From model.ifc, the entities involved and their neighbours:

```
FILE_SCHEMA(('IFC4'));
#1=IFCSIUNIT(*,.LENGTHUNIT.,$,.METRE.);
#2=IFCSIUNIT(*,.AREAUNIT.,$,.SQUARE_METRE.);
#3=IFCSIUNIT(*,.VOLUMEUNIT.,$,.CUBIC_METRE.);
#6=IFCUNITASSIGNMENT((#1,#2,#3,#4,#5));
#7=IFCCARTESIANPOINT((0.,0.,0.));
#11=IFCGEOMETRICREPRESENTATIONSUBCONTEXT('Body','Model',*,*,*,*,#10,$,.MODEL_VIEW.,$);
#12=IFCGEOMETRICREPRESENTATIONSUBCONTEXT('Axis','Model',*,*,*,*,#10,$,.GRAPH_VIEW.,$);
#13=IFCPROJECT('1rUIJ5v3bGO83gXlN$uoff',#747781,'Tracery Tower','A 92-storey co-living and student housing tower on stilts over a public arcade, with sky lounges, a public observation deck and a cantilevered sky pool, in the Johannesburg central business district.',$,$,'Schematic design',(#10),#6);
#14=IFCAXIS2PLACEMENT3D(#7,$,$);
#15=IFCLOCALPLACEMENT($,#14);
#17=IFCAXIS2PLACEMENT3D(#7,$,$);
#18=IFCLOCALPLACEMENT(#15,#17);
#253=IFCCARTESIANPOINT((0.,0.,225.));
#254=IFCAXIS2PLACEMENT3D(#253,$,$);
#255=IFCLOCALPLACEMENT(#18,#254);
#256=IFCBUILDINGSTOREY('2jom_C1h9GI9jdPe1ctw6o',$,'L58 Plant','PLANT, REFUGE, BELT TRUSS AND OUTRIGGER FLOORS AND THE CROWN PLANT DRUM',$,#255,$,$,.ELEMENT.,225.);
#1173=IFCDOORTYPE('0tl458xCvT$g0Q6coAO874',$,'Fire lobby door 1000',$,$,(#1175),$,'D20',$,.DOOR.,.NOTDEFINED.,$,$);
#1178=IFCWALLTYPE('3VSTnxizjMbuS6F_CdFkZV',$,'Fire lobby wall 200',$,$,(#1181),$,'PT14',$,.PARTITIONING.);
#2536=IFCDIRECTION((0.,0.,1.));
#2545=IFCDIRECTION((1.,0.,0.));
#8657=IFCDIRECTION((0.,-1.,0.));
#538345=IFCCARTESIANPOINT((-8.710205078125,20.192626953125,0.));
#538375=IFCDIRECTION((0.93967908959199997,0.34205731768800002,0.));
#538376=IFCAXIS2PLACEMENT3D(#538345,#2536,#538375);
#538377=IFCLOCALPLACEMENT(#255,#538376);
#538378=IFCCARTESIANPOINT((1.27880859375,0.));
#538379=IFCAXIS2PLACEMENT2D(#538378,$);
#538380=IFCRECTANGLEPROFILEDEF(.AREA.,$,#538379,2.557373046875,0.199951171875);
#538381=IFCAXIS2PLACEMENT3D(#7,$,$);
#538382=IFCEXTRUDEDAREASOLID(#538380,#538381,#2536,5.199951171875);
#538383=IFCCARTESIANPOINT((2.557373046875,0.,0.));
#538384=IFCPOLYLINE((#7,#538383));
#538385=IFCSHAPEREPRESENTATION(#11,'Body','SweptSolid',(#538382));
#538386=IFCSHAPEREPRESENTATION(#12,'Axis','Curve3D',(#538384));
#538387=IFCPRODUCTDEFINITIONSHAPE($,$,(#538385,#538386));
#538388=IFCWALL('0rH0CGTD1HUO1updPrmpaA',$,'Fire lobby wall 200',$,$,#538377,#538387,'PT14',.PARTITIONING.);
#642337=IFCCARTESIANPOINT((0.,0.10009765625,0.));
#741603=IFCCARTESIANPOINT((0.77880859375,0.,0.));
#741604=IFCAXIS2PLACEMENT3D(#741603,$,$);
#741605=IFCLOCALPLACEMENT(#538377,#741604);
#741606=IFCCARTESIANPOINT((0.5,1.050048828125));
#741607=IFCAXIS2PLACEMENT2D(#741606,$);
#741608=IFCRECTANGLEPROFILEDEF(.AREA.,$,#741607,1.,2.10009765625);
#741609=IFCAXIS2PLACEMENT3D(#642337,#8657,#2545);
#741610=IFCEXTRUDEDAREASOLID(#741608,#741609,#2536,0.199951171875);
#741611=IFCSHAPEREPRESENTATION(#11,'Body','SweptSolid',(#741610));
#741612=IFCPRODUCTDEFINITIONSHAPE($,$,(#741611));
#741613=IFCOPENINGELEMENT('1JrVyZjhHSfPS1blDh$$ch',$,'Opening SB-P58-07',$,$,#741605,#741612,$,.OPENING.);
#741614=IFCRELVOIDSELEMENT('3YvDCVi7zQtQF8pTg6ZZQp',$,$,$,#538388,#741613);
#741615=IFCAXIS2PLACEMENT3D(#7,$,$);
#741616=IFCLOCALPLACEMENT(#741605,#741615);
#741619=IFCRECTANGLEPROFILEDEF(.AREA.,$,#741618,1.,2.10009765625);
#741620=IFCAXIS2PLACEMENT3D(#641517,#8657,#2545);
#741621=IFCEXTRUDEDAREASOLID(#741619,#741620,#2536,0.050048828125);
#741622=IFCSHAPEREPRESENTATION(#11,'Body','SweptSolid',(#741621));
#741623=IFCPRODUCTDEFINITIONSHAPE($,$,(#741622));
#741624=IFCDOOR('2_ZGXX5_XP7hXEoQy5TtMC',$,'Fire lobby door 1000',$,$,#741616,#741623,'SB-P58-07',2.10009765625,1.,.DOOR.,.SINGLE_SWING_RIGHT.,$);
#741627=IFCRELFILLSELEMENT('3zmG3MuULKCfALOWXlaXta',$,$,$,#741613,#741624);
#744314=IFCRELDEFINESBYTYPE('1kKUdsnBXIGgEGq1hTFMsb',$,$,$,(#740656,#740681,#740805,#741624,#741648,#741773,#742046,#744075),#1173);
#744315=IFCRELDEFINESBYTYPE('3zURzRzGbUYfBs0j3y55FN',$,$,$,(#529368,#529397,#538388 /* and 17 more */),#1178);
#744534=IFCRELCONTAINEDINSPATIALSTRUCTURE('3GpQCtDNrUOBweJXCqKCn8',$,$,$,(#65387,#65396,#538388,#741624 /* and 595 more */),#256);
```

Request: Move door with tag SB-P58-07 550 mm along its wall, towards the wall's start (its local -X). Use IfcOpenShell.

```python
import ifcopenshell
import ifcopenshell.api.geometry
import ifcopenshell.util.placement
import ifcopenshell.util.unit

model = ifcopenshell.open("model.ifc")
unit_scale = ifcopenshell.util.unit.calculate_unit_scale(model)

door = model.by_id(741624)
opening = door.FillsVoids[0].RelatingOpeningElement
wall = opening.VoidsElements[0].RelatingBuildingElement

wall_matrix = ifcopenshell.util.placement.get_local_placement(wall.ObjectPlacement)
shift = wall_matrix[:3, 0] * -0.55 / unit_scale
before = ifcopenshell.util.placement.get_local_placement(door.ObjectPlacement)[:3, 3].copy()

# The door is placed relative to its opening, so it follows when the opening moves.
matrix = ifcopenshell.util.placement.get_local_placement(opening.ObjectPlacement)
matrix[:3, 3] += shift
ifcopenshell.api.geometry.edit_object_placement(
    model, product=opening, matrix=matrix, is_si=False, should_transform_children=True
)

after = ifcopenshell.util.placement.get_local_placement(door.ObjectPlacement)[:3, 3]
print("door moved by", (after - before).round(3) + 0.0)

model.write("model_v2.ifc")
```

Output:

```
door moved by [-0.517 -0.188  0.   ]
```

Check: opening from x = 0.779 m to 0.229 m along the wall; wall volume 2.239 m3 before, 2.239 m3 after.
